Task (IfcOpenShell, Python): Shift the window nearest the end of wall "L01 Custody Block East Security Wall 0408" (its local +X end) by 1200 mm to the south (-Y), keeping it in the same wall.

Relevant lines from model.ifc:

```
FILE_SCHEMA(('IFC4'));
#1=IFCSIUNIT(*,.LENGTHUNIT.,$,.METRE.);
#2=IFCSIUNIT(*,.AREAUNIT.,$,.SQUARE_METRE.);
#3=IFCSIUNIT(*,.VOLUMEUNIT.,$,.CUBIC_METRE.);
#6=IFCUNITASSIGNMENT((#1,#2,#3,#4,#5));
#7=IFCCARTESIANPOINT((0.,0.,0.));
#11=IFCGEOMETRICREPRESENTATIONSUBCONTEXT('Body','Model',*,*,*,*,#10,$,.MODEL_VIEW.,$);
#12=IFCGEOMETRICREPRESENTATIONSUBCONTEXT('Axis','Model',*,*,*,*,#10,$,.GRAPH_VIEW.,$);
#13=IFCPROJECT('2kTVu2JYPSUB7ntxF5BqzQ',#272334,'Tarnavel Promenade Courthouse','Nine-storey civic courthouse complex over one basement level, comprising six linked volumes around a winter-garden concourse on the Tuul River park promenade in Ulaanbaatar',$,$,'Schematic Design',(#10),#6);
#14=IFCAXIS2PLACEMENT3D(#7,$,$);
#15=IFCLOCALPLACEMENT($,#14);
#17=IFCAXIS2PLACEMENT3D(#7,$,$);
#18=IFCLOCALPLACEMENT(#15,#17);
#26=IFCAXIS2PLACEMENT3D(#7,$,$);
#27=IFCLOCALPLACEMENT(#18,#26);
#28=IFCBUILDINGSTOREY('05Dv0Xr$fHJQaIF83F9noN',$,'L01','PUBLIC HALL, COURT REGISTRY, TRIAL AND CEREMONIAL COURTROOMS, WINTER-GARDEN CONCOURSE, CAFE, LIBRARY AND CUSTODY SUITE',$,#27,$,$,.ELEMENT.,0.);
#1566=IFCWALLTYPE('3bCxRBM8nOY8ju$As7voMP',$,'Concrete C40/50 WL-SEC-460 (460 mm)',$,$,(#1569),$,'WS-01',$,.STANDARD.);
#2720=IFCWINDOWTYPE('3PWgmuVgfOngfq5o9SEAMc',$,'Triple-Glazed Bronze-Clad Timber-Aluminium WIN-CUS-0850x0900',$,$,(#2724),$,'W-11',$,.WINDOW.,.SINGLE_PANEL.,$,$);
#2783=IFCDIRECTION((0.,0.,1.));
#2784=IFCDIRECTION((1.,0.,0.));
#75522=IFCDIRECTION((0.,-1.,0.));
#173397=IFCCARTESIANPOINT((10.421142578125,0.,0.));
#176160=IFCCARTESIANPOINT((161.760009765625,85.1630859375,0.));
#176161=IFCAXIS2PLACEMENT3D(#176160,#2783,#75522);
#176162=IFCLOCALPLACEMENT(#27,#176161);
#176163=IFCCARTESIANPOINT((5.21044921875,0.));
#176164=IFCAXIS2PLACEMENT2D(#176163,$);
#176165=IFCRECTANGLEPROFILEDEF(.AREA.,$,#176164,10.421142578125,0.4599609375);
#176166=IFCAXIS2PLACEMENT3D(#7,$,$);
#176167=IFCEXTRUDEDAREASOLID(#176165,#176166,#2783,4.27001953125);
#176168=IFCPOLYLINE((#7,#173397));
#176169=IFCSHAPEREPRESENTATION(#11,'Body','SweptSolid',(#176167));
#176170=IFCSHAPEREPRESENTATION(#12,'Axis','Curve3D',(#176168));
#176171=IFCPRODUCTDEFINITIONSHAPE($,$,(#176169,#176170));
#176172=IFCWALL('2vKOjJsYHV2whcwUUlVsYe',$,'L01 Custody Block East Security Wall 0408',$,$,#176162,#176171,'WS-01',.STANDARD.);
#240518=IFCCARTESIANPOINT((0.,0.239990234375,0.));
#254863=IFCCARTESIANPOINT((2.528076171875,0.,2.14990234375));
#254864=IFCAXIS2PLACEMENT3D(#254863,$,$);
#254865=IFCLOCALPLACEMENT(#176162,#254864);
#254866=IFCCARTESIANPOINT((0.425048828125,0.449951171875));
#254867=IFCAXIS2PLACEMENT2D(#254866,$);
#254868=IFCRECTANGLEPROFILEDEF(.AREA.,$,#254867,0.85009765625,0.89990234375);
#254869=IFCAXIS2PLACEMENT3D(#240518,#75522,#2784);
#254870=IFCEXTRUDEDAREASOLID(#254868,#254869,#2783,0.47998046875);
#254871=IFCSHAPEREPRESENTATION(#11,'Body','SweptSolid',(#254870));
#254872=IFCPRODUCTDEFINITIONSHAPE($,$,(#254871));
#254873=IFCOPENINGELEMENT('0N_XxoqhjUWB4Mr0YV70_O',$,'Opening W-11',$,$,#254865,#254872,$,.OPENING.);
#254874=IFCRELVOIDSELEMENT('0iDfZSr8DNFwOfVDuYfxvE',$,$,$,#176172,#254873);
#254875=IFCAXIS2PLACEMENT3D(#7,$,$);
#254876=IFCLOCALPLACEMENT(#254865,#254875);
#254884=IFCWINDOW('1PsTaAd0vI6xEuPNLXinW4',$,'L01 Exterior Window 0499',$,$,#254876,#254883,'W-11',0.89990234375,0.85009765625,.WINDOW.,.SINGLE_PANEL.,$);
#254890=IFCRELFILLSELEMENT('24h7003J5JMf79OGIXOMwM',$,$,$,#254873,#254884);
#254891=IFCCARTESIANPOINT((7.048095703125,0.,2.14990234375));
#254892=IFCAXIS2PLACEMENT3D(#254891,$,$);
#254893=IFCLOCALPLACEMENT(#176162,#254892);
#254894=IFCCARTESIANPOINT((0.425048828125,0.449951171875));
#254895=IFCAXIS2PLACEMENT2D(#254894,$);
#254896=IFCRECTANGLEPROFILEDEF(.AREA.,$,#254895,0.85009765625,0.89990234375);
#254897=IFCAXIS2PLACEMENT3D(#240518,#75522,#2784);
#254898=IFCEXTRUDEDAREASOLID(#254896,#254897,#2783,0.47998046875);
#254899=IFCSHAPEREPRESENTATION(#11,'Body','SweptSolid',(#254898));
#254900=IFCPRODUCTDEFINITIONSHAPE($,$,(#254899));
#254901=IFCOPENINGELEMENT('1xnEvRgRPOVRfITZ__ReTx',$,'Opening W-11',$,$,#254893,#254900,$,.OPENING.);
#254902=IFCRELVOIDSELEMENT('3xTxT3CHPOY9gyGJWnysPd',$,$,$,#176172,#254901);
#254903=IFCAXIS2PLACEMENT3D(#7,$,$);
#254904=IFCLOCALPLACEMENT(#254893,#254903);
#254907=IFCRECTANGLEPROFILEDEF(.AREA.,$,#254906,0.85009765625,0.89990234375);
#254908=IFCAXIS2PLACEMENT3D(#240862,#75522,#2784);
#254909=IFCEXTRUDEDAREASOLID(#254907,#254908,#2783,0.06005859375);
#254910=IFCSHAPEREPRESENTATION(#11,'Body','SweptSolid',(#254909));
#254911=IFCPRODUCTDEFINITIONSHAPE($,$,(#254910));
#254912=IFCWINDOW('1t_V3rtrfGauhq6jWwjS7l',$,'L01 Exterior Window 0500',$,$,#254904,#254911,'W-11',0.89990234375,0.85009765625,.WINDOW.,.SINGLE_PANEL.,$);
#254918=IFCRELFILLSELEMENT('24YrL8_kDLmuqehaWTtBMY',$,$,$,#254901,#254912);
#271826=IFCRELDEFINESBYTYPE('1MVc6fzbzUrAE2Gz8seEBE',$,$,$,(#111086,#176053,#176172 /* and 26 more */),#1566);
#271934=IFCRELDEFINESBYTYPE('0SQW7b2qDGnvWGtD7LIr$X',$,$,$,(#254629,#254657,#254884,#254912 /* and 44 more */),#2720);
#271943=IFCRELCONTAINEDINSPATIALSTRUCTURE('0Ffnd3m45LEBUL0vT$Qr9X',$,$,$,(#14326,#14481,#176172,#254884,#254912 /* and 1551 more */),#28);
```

```python
import ifcopenshell
import ifcopenshell.api.geometry
import ifcopenshell.util.placement
import ifcopenshell.util.unit

model = ifcopenshell.open("model.ifc")
unit_scale = ifcopenshell.util.unit.calculate_unit_scale(model)

window = model.by_guid("1t_V3rtrfGauhq6jWwjS7l")
opening = window.FillsVoids[0].RelatingOpeningElement
wall = opening.VoidsElements[0].RelatingBuildingElement

wall_matrix = ifcopenshell.util.placement.get_local_placement(wall.ObjectPlacement)
shift = wall_matrix[:3, 0] * 1.2 / unit_scale
before = ifcopenshell.util.placement.get_local_placement(window.ObjectPlacement)[:3, 3].copy()

# The window is placed relative to its opening, so it follows when the opening moves.
matrix = ifcopenshell.util.placement.get_local_placement(opening.ObjectPlacement)
matrix[:3, 3] += shift
ifcopenshell.api.geometry.edit_object_placement(
    model, product=opening, matrix=matrix, is_si=False, should_transform_children=True
)

after = ifcopenshell.util.placement.get_local_placement(window.ObjectPlacement)[:3, 3]
print("window moved by", (after - before).round(3) + 0.0)

model.write("model_edited.ifc")
```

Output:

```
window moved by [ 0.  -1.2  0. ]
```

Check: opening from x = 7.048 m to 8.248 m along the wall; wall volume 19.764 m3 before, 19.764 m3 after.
